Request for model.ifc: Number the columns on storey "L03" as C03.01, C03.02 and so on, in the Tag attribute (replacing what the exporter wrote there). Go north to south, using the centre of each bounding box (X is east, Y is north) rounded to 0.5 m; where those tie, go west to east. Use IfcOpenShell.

First a look at what the model holds.

```python
import ifcopenshell
import ifcopenshell.util.element
import ifcopenshell.util.placement

model = ifcopenshell.open("model.ifc")
print(model.schema)
storey = next(s for s in model.by_type("IfcBuildingStorey") if s.Name == "L03")
columns = [e for e in ifcopenshell.util.element.get_decomposition(storey) if e.is_a("IfcColumn")]
for e in sorted(columns, key=lambda e: e.id()):
    origin = ifcopenshell.util.placement.get_local_placement(e.ObjectPlacement)[:3, 3]
    print(e.id(), e.Tag, e.Name, origin.round(2) + 0.0, sep=" | ")
```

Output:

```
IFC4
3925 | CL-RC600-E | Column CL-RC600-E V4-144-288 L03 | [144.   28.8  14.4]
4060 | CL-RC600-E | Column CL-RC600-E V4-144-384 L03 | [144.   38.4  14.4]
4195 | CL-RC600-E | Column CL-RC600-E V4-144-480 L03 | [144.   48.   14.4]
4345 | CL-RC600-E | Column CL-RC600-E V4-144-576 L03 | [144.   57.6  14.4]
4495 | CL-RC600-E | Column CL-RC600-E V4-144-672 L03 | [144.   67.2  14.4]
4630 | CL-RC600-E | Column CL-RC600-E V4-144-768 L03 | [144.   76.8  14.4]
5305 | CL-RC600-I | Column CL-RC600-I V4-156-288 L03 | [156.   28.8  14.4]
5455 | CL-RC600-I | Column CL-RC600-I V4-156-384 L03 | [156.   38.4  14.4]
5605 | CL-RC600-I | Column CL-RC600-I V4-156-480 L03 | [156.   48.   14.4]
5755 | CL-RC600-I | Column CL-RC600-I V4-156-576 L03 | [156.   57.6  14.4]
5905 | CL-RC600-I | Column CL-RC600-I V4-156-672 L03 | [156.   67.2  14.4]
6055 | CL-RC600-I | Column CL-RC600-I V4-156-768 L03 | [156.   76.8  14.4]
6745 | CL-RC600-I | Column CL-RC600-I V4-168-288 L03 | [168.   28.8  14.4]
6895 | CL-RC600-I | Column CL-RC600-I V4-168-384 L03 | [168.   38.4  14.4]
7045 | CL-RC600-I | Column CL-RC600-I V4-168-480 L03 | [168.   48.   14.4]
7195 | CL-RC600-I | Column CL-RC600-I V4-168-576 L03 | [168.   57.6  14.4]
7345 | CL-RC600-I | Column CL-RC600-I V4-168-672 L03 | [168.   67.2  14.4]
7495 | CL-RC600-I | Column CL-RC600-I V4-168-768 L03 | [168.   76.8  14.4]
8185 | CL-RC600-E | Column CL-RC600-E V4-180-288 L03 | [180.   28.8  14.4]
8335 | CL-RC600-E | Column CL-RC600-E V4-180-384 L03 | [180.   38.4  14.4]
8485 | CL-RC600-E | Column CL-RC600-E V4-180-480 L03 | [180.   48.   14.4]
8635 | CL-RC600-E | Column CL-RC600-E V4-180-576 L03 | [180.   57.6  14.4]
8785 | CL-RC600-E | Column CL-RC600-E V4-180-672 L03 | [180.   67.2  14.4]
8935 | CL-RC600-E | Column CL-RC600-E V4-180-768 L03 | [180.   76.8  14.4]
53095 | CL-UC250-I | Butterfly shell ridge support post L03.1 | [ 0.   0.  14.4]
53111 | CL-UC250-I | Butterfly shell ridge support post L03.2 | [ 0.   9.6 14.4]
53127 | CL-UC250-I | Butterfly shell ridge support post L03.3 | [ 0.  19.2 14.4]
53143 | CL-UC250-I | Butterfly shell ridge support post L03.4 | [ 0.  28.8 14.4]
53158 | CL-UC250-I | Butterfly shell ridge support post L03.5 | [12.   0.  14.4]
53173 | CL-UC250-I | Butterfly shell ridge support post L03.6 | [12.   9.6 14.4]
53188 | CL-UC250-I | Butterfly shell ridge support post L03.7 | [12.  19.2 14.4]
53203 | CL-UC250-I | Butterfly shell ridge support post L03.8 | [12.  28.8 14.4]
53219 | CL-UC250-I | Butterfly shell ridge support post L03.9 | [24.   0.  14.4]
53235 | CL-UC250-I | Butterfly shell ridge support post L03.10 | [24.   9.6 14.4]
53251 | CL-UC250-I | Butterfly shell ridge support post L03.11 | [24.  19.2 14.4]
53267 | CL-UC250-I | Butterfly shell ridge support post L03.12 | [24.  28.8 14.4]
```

```python
import ifcopenshell
import ifcopenshell.geom
import ifcopenshell.util.element
import ifcopenshell.util.shape

model = ifcopenshell.open("model.ifc")
settings = ifcopenshell.geom.settings()
settings.set("use-world-coords", True)


def centre(element):
    shape = ifcopenshell.geom.create_shape(settings, element)
    return ifcopenshell.util.shape.get_bbox_centroid(shape.geometry)


storey = next(s for s in model.by_type("IfcBuildingStorey") if s.Name == "L03")
columns = [e for e in ifcopenshell.util.element.get_decomposition(storey) if e.is_a("IfcColumn")]

# Insertion points can sit at a corner or the storey origin, so sort by the geometry (in metres).
centres = {e: centre(e) for e in columns}
columns.sort(key=lambda e: (-round(centres[e][1] / 0.5), centres[e][0]))

for i, e in enumerate(columns, start=1):
    number = f"C03.{i:02d}"
    e.Tag = number
    print(e.id(), number)

model.write("model_v2.ifc")
```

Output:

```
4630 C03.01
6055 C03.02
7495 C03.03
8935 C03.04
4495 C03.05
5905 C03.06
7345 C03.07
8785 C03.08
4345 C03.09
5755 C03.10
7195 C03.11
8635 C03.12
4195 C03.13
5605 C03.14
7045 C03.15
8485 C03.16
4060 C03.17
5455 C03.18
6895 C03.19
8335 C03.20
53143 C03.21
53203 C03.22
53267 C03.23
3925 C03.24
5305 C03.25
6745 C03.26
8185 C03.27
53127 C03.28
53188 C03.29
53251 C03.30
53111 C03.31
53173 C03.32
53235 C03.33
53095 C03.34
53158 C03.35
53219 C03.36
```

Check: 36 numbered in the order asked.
